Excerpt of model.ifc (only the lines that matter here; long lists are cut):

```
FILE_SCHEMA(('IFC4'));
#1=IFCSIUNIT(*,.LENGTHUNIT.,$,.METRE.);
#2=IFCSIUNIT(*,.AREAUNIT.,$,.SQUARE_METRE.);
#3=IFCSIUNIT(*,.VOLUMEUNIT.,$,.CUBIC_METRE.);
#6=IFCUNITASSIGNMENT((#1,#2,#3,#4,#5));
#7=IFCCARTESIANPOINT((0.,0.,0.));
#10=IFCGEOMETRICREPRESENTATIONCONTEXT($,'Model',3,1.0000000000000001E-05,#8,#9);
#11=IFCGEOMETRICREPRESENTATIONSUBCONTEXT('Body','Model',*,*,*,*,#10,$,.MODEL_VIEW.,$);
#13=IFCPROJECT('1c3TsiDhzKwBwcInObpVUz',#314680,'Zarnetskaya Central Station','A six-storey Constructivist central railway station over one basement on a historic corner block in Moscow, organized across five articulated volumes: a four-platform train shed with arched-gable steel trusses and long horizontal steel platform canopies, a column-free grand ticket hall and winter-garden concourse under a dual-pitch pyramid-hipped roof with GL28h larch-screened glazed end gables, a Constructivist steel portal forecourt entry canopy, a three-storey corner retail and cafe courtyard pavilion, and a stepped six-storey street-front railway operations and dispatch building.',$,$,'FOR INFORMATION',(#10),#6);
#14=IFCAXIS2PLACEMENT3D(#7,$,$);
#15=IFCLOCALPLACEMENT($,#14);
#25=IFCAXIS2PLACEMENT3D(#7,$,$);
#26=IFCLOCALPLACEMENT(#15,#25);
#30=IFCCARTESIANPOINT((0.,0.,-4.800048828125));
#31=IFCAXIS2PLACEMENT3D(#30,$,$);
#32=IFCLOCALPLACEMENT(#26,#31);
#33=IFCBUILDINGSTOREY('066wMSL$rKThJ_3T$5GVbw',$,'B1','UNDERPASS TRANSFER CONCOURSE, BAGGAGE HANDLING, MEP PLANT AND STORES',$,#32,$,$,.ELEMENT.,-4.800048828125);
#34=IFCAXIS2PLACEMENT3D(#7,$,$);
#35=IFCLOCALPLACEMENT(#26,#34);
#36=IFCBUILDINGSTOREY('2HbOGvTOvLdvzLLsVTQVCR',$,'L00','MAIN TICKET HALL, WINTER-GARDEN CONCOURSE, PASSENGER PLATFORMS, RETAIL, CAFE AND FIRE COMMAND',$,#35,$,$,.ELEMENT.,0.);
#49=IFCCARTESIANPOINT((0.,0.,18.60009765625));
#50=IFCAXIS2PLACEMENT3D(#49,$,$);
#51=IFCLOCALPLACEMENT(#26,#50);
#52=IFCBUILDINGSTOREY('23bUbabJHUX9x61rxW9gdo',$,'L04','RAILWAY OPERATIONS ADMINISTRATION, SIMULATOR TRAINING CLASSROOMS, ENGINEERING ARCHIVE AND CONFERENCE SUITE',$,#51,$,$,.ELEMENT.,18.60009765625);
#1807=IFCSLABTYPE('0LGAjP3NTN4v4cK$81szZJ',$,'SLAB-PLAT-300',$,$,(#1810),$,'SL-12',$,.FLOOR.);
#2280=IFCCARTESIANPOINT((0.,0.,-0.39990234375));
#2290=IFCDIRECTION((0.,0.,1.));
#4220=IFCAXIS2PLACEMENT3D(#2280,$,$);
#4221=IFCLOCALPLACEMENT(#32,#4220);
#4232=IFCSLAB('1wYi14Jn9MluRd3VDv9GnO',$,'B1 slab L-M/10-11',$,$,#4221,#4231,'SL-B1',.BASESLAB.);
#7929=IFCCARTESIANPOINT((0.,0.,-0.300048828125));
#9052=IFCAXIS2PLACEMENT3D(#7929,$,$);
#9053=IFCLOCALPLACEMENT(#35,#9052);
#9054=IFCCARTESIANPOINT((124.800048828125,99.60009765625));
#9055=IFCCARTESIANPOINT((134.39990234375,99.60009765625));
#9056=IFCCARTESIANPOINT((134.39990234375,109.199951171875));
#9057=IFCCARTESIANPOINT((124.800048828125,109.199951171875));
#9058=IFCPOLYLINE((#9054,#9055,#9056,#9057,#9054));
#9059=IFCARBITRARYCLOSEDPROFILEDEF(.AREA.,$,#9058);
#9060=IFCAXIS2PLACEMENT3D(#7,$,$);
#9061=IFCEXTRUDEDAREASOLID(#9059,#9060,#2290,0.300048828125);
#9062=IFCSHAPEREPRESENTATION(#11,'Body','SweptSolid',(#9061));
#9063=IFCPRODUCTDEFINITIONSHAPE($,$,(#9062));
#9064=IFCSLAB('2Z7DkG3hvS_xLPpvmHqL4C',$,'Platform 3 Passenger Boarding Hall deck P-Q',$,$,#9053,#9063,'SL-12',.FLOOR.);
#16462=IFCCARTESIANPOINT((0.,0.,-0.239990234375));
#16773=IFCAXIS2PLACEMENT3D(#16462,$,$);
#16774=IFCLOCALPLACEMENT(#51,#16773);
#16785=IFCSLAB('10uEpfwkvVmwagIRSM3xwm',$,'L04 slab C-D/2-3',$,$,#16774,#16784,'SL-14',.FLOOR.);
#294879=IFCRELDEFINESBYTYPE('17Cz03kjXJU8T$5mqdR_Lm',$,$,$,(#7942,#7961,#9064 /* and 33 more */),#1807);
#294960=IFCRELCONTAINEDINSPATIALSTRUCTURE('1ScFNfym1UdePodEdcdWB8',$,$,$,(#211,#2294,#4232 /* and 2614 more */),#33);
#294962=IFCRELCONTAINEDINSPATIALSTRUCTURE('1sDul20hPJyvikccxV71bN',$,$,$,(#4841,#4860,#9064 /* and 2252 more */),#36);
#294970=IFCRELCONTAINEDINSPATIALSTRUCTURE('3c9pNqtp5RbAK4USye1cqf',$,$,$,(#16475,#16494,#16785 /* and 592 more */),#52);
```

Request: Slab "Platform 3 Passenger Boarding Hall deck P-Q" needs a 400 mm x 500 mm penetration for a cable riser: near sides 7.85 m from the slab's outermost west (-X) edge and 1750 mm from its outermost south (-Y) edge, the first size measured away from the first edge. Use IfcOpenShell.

```python
import numpy as np
import ifcopenshell
import ifcopenshell.api.feature
import ifcopenshell.api.geometry
import ifcopenshell.api.root
import ifcopenshell.geom
import ifcopenshell.util.placement
import ifcopenshell.util.representation
import ifcopenshell.util.shape
import ifcopenshell.util.unit

model = ifcopenshell.open("model.ifc")
unit_scale = ifcopenshell.util.unit.calculate_unit_scale(model)
settings = ifcopenshell.geom.settings()


def volume(element):
    """Net volume in cubic metres, openings subtracted."""
    shape = ifcopenshell.geom.create_shape(settings, element)
    return ifcopenshell.util.shape.get_volume(shape.geometry)


slab = model.by_guid("2Z7DkG3hvS_xLPpvmHqL4C")
before = volume(slab)

# Extent in the slab's own axes, in metres. The edges named are its -X and -Y sides.
slab_shape = ifcopenshell.geom.create_shape(settings, slab)
vertices = ifcopenshell.util.shape.get_vertices(slab_shape.geometry)
x_min, y_min, bottom = vertices.min(axis=0)
top = vertices[:, 2].max()

opening = ifcopenshell.api.root.create_entity(model, ifc_class="IfcOpeningElement", name="Cable riser opening", predefined_type="OPENING")
context = ifcopenshell.util.representation.get_context(model, "Model", "Body", "MODEL_VIEW")
width, depth = 0.4, 0.5
outline = [(0.0, 0.0), (width, 0.0), (width, depth), (0.0, depth), (0.0, 0.0)]
# Overshoot both faces by 50 mm so the cut is clean.
shape = ifcopenshell.api.geometry.add_slab_representation(
    model, context=context, depth=top - bottom + 0.1, polyline=outline
)
ifcopenshell.api.geometry.assign_representation(model, product=opening, representation=shape)

matrix = ifcopenshell.util.placement.get_local_placement(slab.ObjectPlacement)
matrix[:, 3] = matrix @ np.append(np.array([x_min + 7.85, y_min + 1.75, bottom - 0.05]) / unit_scale, 1.0)
ifcopenshell.api.geometry.edit_object_placement(model, product=opening, matrix=matrix, is_si=False)
ifcopenshell.api.feature.add_feature(model, feature=opening, element=slab)

after = volume(slab)

print(f"slab volume {before:.3f} -> {after:.3f} m3")

model.write("model_rev.ifc")
```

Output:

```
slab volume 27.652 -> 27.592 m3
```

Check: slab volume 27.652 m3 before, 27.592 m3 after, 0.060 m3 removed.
